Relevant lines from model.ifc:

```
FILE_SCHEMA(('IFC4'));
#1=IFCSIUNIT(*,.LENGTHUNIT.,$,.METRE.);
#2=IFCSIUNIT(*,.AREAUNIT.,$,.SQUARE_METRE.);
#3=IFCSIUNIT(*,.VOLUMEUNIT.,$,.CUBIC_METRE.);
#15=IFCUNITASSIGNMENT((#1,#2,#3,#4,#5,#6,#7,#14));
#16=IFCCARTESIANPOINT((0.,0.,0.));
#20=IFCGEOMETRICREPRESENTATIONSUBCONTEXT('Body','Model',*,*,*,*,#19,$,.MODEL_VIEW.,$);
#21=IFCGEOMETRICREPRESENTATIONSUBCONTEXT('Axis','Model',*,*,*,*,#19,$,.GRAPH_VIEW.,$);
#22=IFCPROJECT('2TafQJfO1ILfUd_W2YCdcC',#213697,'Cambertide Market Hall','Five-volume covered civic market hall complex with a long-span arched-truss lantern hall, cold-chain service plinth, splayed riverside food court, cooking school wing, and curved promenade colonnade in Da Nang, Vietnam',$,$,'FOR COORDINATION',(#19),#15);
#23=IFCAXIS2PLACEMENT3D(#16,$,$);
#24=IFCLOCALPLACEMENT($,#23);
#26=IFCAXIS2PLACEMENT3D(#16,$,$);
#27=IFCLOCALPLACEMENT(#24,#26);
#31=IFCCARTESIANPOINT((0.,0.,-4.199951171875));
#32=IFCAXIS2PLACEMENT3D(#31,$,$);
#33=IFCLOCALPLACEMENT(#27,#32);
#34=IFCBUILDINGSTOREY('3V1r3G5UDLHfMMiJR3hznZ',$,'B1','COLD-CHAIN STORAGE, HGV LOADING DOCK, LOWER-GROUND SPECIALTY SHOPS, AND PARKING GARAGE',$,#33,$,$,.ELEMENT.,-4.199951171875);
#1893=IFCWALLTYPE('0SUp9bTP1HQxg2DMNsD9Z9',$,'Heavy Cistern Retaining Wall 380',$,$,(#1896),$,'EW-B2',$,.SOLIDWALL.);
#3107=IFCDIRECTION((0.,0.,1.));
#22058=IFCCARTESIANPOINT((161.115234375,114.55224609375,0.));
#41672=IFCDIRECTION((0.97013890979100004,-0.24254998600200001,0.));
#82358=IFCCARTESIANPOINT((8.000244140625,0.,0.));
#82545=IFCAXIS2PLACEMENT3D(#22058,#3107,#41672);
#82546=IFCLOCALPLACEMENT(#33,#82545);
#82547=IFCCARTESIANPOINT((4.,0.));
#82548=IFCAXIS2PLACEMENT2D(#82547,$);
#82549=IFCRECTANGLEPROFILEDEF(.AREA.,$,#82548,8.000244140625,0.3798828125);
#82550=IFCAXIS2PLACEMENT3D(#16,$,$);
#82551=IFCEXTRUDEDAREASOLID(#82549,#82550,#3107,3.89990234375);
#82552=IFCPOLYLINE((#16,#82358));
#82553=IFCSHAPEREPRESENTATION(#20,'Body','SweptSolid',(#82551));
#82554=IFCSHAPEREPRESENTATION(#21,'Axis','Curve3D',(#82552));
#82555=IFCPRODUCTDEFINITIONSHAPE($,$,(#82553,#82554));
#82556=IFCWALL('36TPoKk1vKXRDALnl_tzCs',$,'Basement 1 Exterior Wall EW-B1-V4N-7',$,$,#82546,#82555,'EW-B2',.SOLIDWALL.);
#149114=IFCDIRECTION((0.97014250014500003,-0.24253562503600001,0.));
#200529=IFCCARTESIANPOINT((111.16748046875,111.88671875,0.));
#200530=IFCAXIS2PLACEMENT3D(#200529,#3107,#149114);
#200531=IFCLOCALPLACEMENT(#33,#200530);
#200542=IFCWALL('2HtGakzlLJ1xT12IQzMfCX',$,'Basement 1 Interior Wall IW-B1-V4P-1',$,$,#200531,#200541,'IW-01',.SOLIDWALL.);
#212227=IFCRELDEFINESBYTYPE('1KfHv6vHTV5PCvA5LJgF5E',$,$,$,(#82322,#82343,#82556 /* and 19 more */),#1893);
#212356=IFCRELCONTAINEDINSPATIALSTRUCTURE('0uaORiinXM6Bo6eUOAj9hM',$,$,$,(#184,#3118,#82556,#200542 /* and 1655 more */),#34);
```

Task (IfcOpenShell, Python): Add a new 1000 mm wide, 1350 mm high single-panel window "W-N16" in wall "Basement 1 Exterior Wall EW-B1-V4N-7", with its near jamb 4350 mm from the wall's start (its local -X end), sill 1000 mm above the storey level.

```python
import numpy as np
import ifcopenshell
import ifcopenshell.api.feature
import ifcopenshell.api.geometry
import ifcopenshell.api.root
import ifcopenshell.api.spatial
import ifcopenshell.geom
import ifcopenshell.util.element
import ifcopenshell.util.placement
import ifcopenshell.util.representation
import ifcopenshell.util.shape
import ifcopenshell.util.unit

model = ifcopenshell.open("model.ifc")
unit_scale = ifcopenshell.util.unit.calculate_unit_scale(model)
settings = ifcopenshell.geom.settings()


def volume(element):
    """Net volume in cubic metres, openings subtracted."""
    shape = ifcopenshell.geom.create_shape(settings, element)
    return ifcopenshell.util.shape.get_volume(shape.geometry)


wall = model.by_guid("36TPoKk1vKXRDALnl_tzCs")
storey = ifcopenshell.util.element.get_container(wall, ifc_class="IfcBuildingStorey")
context = ifcopenshell.util.representation.get_context(model, "Model", "Body", "MODEL_VIEW")
before = volume(wall)

width, height, from_end, sill = 1, 1.35, 4.35, 1  # metres

# The wall runs along its own X axis, and the end named is its -X end.
wall_shape = ifcopenshell.geom.create_shape(settings, wall)
x, y, z = ifcopenshell.util.shape.get_vertices(wall_shape.geometry).T
start = x.min() + from_end
face, thickness = float(y.min()), float(y.max() - y.min())
wall_matrix = ifcopenshell.util.placement.get_local_placement(wall.ObjectPlacement)
level = ifcopenshell.util.placement.get_local_placement(storey.ObjectPlacement)[2, 3]


def in_wall(x, y):
    """Placement at x, y metres in the wall's axes, at sill height."""
    matrix = wall_matrix.copy()
    matrix[:, 3] = wall_matrix @ np.array([x / unit_scale, y / unit_scale, 0.0, 1.0])
    matrix[2, 3] = level + sill / unit_scale
    return matrix


# Opening: a box that overshoots both wall faces by 50 mm.
opening = ifcopenshell.api.root.create_entity(model, ifc_class="IfcOpeningElement", predefined_type="OPENING")
box = ifcopenshell.api.geometry.add_wall_representation(
    model, context=context, length=width, height=height, thickness=thickness + 0.1
)
ifcopenshell.api.geometry.assign_representation(model, product=opening, representation=box)
ifcopenshell.api.geometry.edit_object_placement(model, product=opening, matrix=in_wall(start, face - 0.05), is_si=False)
ifcopenshell.api.feature.add_feature(model, feature=opening, element=wall)

window = ifcopenshell.api.root.create_entity(model, ifc_class="IfcWindow", name="W-N16", predefined_type="WINDOW")
window.OverallWidth, window.OverallHeight = width / unit_scale, height / unit_scale
window.PartitioningType = "SINGLE_PANEL"
body = ifcopenshell.api.geometry.add_window_representation(
    model,
    context=context,
    overall_width=window.OverallWidth,
    overall_height=window.OverallHeight,
    partition_type="SINGLE_PANEL",
)
ifcopenshell.api.geometry.assign_representation(model, product=window, representation=body)
ifcopenshell.api.spatial.assign_container(model, products=[window], relating_structure=storey)
ifcopenshell.api.feature.add_filling(model, opening=opening, element=window)

# Centre the window in the wall's thickness.
ifcopenshell.api.geometry.edit_object_placement(model, product=window, matrix=in_wall(start, face), is_si=False)
window_shape = ifcopenshell.geom.create_shape(settings, window)
depth = ifcopenshell.util.shape.get_vertices(window_shape.geometry)[:, 1]
offset = face + thickness / 2 - (depth.min() + depth.max()) / 2
ifcopenshell.api.geometry.edit_object_placement(model, product=window, matrix=in_wall(start, offset), is_si=False)

after = volume(wall)

print(f"wall volume {before:.3f} -> {after:.3f} m3")

model.write("model-out.ifc")
```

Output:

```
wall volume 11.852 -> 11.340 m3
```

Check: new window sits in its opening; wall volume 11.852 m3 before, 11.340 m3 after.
